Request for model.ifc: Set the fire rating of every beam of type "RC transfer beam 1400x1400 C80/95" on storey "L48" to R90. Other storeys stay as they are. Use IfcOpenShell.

First a look at what the model holds.

```python
import ifcopenshell
import ifcopenshell.util.element

model = ifcopenshell.open("model.ifc")
print(model.schema)
storey = next(s for s in model.by_type("IfcBuildingStorey") if s.Name == "L48")
beams = [e for e in ifcopenshell.util.element.get_decomposition(storey) if e.is_a("IfcBeam")]
seen = {}
for e in beams:
    element_type = ifcopenshell.util.element.get_type(e)
    key = (element_type.Name if element_type != e and element_type else None, ifcopenshell.util.element.get_pset(e, "Pset_BeamCommon", "FireRating"))
    seen[key] = seen.get(key, 0) + 1
for (name, value), count in sorted(seen.items(), key=str):
    print(count, "x", name, "|", value)
```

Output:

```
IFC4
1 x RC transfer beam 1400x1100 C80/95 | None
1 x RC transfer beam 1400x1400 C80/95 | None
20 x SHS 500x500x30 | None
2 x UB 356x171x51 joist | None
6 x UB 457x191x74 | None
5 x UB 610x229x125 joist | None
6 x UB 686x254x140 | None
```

```python
import ifcopenshell
import ifcopenshell.api.pset
import ifcopenshell.util.element

model = ifcopenshell.open("model.ifc")

storey = next(s for s in model.by_type("IfcBuildingStorey") if s.Name == "L48")
beams = [e for e in ifcopenshell.util.element.get_decomposition(storey) if e.is_a("IfcBeam")]

count = 0
for e in beams:
    element_type = ifcopenshell.util.element.get_type(e)
    if element_type in (None, e) or element_type.Name != "RC transfer beam 1400x1400 C80/95":
        continue
    found = ifcopenshell.util.element.get_pset(e, "Pset_BeamCommon", should_inherit=False)
    if found:
        pset = model.by_id(found["id"])
        if len(ifcopenshell.util.element.get_elements_by_pset(pset)) > 1:
            pset = ifcopenshell.api.pset.unshare_pset(model, products=[e], pset=pset)[0]
    else:
        pset = ifcopenshell.api.pset.add_pset(model, product=e, name="Pset_BeamCommon")
    ifcopenshell.api.pset.edit_pset(model, pset=pset, properties={"FireRating": "R90"})
    count += 1

print(count, "beams updated")

model.write("model_edited.ifc")
```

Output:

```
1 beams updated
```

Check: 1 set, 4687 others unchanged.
